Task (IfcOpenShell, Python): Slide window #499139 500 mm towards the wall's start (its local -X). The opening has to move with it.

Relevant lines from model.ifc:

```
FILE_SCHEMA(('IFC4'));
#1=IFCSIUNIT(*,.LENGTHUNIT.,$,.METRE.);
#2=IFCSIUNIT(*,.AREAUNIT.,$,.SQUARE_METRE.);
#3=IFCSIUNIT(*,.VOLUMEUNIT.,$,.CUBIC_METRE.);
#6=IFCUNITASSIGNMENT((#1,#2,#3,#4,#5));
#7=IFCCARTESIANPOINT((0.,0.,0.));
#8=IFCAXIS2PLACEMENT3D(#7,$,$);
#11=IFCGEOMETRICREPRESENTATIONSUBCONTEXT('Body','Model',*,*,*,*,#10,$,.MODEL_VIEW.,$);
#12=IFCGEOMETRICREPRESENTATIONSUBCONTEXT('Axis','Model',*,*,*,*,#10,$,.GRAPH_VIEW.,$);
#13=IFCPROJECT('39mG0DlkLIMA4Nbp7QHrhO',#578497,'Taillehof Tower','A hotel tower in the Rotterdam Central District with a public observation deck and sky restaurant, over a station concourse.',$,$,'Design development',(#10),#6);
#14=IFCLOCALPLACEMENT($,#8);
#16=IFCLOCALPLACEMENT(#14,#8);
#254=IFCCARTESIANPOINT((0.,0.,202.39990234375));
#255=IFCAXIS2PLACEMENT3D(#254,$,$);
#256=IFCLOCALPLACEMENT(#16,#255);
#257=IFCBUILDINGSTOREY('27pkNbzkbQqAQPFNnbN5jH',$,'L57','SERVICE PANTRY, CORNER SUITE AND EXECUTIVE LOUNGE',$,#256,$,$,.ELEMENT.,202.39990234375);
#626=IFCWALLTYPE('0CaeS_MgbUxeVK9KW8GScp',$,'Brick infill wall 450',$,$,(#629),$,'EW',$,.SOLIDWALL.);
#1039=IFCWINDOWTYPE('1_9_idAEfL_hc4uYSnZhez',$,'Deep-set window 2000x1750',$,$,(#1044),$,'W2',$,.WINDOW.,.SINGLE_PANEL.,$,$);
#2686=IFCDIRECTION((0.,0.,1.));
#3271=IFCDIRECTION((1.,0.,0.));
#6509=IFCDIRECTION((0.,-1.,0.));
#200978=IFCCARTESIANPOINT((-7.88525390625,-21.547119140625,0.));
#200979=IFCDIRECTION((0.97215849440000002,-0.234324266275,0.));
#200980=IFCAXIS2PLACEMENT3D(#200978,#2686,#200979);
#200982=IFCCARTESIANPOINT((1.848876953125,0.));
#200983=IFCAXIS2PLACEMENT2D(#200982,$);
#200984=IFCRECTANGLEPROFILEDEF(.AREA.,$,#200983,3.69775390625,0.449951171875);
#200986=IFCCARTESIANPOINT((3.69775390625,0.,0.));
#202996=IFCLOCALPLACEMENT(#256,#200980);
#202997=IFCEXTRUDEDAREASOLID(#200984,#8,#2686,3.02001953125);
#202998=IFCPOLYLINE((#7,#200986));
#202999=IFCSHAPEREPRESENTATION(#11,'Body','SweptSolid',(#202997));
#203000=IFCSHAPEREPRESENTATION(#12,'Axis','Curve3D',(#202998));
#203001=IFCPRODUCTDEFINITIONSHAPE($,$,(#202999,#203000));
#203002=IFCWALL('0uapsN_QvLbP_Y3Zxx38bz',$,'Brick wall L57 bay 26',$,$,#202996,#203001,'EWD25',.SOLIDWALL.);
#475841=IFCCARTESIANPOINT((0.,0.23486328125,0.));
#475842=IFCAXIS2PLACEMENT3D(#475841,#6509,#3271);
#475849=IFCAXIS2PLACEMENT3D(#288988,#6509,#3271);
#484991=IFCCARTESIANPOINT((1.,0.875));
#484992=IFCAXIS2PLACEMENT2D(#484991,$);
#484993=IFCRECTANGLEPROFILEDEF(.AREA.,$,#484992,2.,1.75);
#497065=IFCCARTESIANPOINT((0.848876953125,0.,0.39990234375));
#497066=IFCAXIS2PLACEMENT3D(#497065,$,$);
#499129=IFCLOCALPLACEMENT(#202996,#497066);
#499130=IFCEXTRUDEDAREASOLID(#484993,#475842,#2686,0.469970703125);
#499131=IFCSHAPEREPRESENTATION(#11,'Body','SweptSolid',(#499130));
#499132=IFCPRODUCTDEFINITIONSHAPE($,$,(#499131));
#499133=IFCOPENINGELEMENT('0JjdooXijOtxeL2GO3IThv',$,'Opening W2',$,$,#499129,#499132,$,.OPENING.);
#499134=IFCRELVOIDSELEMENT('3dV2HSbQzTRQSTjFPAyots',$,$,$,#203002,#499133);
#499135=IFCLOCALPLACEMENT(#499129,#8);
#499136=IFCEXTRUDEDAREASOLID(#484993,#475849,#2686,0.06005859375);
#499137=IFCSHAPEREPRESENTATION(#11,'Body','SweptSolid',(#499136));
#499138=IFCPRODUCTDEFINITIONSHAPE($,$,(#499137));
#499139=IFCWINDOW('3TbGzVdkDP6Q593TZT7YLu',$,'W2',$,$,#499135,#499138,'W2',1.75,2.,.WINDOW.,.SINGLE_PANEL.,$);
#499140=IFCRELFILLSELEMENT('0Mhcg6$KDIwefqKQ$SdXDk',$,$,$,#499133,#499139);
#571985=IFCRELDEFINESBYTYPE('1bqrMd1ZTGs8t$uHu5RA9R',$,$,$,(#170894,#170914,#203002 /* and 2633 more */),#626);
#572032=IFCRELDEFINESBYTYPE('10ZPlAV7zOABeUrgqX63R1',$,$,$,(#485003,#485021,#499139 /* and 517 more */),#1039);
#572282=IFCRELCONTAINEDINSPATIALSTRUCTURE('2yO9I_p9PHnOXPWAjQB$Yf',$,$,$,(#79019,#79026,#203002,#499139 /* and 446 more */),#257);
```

```python
import ifcopenshell
import ifcopenshell.api.geometry
import ifcopenshell.util.placement
import ifcopenshell.util.unit

model = ifcopenshell.open("model.ifc")
unit_scale = ifcopenshell.util.unit.calculate_unit_scale(model)

window = model.by_guid("3TbGzVdkDP6Q593TZT7YLu")
opening = window.FillsVoids[0].RelatingOpeningElement
wall = opening.VoidsElements[0].RelatingBuildingElement

wall_matrix = ifcopenshell.util.placement.get_local_placement(wall.ObjectPlacement)
shift = wall_matrix[:3, 0] * -0.5 / unit_scale
before = ifcopenshell.util.placement.get_local_placement(window.ObjectPlacement)[:3, 3].copy()

# The window is placed relative to its opening, so it follows when the opening moves.
matrix = ifcopenshell.util.placement.get_local_placement(opening.ObjectPlacement)
matrix[:3, 3] += shift
ifcopenshell.api.geometry.edit_object_placement(
    model, product=opening, matrix=matrix, is_si=False, should_transform_children=True
)

after = ifcopenshell.util.placement.get_local_placement(window.ObjectPlacement)[:3, 3]
print("window moved by", (after - before).round(3) + 0.0)

model.write("model_edited.ifc")
```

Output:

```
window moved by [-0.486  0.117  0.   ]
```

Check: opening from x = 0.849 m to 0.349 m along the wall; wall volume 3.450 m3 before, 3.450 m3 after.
